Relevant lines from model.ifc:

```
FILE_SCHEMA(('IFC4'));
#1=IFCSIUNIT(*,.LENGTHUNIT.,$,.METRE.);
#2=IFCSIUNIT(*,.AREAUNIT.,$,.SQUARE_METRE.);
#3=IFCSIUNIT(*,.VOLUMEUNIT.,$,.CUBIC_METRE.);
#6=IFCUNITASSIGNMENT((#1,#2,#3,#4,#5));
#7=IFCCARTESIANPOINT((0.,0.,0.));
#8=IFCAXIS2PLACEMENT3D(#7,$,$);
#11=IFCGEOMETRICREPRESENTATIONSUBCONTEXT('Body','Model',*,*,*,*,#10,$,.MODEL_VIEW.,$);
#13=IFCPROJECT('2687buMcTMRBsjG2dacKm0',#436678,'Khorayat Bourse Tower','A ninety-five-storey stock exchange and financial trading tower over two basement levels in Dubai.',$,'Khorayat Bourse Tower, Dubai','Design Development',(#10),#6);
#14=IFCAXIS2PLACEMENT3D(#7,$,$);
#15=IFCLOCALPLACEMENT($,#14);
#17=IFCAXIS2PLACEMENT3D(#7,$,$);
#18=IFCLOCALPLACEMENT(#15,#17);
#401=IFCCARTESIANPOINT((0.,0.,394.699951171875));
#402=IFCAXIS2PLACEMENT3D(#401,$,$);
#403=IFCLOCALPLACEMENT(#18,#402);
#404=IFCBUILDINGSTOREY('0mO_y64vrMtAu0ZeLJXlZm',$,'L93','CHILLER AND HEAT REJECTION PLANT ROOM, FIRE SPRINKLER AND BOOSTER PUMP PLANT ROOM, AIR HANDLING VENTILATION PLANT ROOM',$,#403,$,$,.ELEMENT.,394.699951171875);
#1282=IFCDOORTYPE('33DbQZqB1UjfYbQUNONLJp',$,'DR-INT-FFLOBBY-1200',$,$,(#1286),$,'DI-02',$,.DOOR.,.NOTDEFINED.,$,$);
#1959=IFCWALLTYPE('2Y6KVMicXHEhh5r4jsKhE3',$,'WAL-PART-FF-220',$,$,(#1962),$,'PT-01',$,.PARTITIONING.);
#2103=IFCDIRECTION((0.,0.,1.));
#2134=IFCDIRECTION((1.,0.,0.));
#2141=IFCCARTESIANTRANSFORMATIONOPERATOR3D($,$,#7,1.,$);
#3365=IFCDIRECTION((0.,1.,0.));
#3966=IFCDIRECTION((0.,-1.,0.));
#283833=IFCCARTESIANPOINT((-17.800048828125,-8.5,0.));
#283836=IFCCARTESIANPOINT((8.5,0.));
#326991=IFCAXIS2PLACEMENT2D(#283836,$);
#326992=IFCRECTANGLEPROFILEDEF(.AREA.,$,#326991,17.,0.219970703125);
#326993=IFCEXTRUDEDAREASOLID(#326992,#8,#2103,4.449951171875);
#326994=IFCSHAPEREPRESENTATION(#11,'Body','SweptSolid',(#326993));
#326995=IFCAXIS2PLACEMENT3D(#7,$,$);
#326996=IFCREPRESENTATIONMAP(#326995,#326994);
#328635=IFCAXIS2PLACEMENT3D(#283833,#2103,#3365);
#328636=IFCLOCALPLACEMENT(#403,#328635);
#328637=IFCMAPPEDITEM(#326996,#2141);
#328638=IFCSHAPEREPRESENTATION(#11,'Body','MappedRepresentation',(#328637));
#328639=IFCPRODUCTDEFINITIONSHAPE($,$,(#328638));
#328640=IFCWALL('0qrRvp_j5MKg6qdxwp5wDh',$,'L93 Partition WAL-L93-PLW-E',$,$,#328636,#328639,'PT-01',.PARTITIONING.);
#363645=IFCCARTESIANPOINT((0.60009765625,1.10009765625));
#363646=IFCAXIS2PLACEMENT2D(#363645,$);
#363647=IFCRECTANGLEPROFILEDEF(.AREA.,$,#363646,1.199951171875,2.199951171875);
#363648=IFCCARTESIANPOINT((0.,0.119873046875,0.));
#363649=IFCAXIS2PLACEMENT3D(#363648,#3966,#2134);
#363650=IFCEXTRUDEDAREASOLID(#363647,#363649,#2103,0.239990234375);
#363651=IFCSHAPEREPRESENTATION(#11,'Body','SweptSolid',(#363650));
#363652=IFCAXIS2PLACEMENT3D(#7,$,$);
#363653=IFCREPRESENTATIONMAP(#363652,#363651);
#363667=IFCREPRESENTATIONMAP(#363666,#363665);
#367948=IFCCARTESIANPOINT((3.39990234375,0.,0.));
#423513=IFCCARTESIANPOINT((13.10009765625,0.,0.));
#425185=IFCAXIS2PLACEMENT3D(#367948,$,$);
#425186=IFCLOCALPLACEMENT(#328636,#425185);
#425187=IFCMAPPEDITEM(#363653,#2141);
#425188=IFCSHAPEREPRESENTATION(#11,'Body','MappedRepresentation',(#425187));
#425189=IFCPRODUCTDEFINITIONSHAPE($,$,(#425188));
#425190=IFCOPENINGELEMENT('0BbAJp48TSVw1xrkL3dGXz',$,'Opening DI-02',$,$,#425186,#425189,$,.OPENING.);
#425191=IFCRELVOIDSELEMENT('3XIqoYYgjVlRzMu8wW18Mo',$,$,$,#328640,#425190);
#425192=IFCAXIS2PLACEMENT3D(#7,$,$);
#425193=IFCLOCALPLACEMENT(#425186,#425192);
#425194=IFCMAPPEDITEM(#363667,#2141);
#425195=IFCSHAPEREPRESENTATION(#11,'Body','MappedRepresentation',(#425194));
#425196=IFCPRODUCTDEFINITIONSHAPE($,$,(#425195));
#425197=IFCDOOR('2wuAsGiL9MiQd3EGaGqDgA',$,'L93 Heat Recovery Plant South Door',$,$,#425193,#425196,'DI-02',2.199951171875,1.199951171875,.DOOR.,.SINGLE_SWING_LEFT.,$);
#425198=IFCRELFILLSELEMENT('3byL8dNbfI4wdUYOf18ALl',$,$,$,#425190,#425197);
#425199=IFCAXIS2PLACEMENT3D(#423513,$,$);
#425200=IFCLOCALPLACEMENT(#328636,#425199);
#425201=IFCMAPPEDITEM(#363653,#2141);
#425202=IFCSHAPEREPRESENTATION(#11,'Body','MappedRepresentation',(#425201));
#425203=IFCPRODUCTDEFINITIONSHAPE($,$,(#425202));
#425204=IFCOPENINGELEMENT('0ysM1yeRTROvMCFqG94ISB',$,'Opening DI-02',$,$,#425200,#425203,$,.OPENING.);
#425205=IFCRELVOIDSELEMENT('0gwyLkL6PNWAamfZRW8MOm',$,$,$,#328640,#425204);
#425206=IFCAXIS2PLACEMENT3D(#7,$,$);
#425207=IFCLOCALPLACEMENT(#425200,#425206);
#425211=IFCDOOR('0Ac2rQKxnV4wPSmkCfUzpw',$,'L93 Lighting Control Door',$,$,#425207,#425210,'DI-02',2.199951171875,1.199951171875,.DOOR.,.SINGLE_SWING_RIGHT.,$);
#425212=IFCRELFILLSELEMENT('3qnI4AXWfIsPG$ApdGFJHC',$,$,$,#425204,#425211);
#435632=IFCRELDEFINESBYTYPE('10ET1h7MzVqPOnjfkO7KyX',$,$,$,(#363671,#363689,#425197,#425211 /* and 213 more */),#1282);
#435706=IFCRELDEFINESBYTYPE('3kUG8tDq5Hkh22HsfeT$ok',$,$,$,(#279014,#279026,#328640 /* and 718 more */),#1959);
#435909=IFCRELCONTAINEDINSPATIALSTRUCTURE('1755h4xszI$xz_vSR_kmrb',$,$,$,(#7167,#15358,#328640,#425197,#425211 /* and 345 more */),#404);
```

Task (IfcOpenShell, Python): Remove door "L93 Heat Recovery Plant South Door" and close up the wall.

```python
import ifcopenshell
import ifcopenshell.api.feature
import ifcopenshell.api.root
import ifcopenshell.geom
import ifcopenshell.util.shape

model = ifcopenshell.open("model.ifc")
settings = ifcopenshell.geom.settings()


def volume(element):
    """Net volume in cubic metres, openings subtracted."""
    shape = ifcopenshell.geom.create_shape(settings, element)
    return ifcopenshell.util.shape.get_volume(shape.geometry)


door = model.by_id(425197)
opening = door.FillsVoids[0].RelatingOpeningElement
wall = opening.VoidsElements[0].RelatingBuildingElement
before = volume(wall)

ifcopenshell.api.root.remove_product(model, product=door)
ifcopenshell.api.feature.remove_feature(model, feature=opening)

after = volume(wall)

print(f"wall volume {before:.3f} -> {after:.3f} m3")

model.write("model_updated.ifc")
```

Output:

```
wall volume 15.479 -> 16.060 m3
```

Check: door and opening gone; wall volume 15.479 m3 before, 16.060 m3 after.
